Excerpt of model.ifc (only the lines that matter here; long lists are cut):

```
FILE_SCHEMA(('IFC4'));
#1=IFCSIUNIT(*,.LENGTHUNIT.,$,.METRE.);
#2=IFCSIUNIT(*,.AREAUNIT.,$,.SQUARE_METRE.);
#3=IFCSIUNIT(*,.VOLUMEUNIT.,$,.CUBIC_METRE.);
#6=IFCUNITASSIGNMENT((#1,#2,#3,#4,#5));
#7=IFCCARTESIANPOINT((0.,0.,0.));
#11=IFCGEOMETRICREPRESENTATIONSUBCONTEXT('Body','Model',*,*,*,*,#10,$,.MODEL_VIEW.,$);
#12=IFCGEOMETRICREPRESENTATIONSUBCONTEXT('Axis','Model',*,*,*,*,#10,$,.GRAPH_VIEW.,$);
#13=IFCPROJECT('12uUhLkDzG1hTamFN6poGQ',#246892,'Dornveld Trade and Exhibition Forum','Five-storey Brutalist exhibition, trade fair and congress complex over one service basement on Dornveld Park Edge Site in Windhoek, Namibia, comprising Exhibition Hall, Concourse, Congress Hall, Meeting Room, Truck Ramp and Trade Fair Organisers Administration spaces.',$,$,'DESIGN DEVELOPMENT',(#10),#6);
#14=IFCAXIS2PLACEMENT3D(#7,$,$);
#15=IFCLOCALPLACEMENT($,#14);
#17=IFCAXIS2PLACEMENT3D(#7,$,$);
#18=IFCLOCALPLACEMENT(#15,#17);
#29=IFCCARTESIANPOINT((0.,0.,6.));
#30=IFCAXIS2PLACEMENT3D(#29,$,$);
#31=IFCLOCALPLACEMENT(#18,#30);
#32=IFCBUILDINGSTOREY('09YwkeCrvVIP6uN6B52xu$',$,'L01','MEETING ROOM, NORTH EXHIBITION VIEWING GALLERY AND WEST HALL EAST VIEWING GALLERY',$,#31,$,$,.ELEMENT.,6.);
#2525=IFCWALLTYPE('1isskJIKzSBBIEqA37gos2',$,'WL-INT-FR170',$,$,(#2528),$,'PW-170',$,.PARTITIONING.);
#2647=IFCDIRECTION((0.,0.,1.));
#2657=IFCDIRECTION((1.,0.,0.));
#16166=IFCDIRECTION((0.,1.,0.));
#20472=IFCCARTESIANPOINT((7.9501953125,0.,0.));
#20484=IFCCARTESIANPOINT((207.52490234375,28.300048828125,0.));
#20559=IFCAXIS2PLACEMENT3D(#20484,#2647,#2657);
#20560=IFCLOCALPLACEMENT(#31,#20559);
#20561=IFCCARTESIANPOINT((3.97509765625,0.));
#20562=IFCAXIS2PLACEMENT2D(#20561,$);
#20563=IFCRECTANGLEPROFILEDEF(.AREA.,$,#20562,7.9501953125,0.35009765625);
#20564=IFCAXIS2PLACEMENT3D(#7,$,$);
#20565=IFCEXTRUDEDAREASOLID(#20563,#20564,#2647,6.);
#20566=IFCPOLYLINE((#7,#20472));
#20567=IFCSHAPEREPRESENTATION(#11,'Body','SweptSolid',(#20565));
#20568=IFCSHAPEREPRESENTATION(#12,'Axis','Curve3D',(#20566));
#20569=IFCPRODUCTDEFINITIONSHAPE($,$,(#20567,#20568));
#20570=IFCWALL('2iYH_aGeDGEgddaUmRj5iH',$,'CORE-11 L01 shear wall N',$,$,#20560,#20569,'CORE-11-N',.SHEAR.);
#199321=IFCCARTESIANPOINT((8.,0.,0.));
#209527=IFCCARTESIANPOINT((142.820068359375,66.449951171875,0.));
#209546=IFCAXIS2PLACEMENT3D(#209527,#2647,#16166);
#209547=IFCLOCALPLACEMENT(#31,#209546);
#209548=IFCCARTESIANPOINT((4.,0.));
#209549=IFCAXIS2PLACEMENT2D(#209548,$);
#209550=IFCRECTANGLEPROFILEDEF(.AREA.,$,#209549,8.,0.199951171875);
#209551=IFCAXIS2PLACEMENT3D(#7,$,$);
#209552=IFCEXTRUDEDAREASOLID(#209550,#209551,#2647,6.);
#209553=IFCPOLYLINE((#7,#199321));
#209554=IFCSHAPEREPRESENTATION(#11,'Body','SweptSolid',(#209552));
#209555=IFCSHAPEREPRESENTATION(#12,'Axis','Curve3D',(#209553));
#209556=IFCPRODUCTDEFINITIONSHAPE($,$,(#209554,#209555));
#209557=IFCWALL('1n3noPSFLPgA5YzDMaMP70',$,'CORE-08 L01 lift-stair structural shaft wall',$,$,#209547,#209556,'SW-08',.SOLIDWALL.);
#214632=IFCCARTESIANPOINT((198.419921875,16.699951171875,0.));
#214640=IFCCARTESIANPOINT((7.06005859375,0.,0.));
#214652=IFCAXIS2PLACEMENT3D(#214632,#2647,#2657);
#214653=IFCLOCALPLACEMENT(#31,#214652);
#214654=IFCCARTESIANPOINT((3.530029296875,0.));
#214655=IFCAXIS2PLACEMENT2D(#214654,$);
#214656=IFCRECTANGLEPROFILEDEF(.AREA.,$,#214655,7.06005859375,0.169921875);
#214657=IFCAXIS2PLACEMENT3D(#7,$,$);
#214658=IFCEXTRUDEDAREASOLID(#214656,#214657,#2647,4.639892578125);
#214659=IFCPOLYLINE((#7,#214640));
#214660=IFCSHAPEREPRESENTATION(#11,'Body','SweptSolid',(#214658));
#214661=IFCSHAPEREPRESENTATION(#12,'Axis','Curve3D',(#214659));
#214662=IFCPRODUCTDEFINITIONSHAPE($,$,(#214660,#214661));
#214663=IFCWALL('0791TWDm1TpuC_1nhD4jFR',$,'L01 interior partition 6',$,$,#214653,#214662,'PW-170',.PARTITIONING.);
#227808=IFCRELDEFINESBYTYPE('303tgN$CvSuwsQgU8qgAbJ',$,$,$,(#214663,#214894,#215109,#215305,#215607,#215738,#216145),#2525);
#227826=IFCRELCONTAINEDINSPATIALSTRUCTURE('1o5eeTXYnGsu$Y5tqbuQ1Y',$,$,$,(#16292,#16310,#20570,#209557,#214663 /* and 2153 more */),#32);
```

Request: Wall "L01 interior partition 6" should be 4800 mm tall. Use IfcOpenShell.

```python
import ifcopenshell
import ifcopenshell.geom
import ifcopenshell.util.representation
import ifcopenshell.util.shape

model = ifcopenshell.open("model.ifc")
settings = ifcopenshell.geom.settings()


def volume(element):
    """Net volume in cubic metres, openings subtracted."""
    shape = ifcopenshell.geom.create_shape(settings, element)
    return ifcopenshell.util.shape.get_volume(shape.geometry)


wall = model.by_guid("0791TWDm1TpuC_1nhD4jFR")
before = volume(wall)

body = ifcopenshell.util.representation.get_representation(wall, "Model", "Body")
solid = body.Items[0]
old_height = solid.Depth
solid.Depth = 4.8
after = volume(wall)

print(f"height {old_height:g} -> {solid.Depth:g}, volume {before:.3f} -> {after:.3f} m3")

model.write("model_updated.ifc")
```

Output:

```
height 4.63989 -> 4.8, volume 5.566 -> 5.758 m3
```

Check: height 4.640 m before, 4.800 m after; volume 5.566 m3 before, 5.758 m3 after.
